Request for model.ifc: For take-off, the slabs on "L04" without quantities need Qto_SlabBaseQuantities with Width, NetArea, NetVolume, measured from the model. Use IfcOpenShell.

First a look at what the model holds.

```python
import ifcopenshell
import ifcopenshell.util.element
import ifcopenshell.util.unit

model = ifcopenshell.open("model.ifc")
print(model.schema)
for unit_type in ("LENGTHUNIT", "AREAUNIT", "VOLUMEUNIT"):
    print(unit_type, ifcopenshell.util.unit.calculate_unit_scale(model, unit_type))
storey = next(s for s in model.by_type("IfcBuildingStorey") if s.Name == "L04")
slabs = [e for e in ifcopenshell.util.element.get_decomposition(storey) if e.is_a("IfcSlab")]
for e in sorted(slabs, key=lambda e: e.id()):
    print(e.id(), e.is_a(), e.Name, list(ifcopenshell.util.element.get_psets(e, qtos_only=True)), sep=" | ")
```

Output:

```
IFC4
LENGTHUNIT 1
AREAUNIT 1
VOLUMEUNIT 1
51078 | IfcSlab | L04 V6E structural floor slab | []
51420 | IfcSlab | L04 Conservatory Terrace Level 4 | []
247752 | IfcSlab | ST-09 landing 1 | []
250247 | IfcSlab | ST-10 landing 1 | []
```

```python
import ifcopenshell
import ifcopenshell.api.pset
import ifcopenshell.geom
import ifcopenshell.util.element
import ifcopenshell.util.shape
import ifcopenshell.util.unit

model = ifcopenshell.open("model.ifc")
unit_scale = ifcopenshell.util.unit.calculate_unit_scale(model)
area_scale = ifcopenshell.util.unit.calculate_unit_scale(model, "AREAUNIT")
volume_scale = ifcopenshell.util.unit.calculate_unit_scale(model, "VOLUMEUNIT")
settings = ifcopenshell.geom.settings()

storey = next(s for s in model.by_type("IfcBuildingStorey") if s.Name == "L04")
slabs = [e for e in ifcopenshell.util.element.get_decomposition(storey) if e.is_a("IfcSlab")]

for e in sorted(slabs, key=lambda e: e.id()):
    if ifcopenshell.util.element.get_psets(e, qtos_only=True, should_inherit=False):
        continue
    # Geometry comes back in metres, in the element's own axes.
    shape = ifcopenshell.geom.create_shape(settings, e)
    values = {
        "Width": ifcopenshell.util.shape.get_z(shape.geometry) / unit_scale,
        "NetArea": ifcopenshell.util.shape.get_footprint_area(shape.geometry) / area_scale,
        "NetVolume": ifcopenshell.util.shape.get_volume(shape.geometry) / volume_scale,
    }
    qto = ifcopenshell.api.pset.add_qto(model, product=e, name="Qto_SlabBaseQuantities")
    ifcopenshell.api.pset.edit_qto(model, qto=qto, properties=values)
    print(e.id(), {k: round(v, 3) for k, v in values.items()})

model.write("model-out.ifc")
```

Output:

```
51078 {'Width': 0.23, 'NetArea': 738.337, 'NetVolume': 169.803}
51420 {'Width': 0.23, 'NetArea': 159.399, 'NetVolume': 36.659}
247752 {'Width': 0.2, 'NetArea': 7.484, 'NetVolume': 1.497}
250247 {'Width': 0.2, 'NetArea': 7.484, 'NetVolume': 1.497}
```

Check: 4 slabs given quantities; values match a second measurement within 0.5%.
